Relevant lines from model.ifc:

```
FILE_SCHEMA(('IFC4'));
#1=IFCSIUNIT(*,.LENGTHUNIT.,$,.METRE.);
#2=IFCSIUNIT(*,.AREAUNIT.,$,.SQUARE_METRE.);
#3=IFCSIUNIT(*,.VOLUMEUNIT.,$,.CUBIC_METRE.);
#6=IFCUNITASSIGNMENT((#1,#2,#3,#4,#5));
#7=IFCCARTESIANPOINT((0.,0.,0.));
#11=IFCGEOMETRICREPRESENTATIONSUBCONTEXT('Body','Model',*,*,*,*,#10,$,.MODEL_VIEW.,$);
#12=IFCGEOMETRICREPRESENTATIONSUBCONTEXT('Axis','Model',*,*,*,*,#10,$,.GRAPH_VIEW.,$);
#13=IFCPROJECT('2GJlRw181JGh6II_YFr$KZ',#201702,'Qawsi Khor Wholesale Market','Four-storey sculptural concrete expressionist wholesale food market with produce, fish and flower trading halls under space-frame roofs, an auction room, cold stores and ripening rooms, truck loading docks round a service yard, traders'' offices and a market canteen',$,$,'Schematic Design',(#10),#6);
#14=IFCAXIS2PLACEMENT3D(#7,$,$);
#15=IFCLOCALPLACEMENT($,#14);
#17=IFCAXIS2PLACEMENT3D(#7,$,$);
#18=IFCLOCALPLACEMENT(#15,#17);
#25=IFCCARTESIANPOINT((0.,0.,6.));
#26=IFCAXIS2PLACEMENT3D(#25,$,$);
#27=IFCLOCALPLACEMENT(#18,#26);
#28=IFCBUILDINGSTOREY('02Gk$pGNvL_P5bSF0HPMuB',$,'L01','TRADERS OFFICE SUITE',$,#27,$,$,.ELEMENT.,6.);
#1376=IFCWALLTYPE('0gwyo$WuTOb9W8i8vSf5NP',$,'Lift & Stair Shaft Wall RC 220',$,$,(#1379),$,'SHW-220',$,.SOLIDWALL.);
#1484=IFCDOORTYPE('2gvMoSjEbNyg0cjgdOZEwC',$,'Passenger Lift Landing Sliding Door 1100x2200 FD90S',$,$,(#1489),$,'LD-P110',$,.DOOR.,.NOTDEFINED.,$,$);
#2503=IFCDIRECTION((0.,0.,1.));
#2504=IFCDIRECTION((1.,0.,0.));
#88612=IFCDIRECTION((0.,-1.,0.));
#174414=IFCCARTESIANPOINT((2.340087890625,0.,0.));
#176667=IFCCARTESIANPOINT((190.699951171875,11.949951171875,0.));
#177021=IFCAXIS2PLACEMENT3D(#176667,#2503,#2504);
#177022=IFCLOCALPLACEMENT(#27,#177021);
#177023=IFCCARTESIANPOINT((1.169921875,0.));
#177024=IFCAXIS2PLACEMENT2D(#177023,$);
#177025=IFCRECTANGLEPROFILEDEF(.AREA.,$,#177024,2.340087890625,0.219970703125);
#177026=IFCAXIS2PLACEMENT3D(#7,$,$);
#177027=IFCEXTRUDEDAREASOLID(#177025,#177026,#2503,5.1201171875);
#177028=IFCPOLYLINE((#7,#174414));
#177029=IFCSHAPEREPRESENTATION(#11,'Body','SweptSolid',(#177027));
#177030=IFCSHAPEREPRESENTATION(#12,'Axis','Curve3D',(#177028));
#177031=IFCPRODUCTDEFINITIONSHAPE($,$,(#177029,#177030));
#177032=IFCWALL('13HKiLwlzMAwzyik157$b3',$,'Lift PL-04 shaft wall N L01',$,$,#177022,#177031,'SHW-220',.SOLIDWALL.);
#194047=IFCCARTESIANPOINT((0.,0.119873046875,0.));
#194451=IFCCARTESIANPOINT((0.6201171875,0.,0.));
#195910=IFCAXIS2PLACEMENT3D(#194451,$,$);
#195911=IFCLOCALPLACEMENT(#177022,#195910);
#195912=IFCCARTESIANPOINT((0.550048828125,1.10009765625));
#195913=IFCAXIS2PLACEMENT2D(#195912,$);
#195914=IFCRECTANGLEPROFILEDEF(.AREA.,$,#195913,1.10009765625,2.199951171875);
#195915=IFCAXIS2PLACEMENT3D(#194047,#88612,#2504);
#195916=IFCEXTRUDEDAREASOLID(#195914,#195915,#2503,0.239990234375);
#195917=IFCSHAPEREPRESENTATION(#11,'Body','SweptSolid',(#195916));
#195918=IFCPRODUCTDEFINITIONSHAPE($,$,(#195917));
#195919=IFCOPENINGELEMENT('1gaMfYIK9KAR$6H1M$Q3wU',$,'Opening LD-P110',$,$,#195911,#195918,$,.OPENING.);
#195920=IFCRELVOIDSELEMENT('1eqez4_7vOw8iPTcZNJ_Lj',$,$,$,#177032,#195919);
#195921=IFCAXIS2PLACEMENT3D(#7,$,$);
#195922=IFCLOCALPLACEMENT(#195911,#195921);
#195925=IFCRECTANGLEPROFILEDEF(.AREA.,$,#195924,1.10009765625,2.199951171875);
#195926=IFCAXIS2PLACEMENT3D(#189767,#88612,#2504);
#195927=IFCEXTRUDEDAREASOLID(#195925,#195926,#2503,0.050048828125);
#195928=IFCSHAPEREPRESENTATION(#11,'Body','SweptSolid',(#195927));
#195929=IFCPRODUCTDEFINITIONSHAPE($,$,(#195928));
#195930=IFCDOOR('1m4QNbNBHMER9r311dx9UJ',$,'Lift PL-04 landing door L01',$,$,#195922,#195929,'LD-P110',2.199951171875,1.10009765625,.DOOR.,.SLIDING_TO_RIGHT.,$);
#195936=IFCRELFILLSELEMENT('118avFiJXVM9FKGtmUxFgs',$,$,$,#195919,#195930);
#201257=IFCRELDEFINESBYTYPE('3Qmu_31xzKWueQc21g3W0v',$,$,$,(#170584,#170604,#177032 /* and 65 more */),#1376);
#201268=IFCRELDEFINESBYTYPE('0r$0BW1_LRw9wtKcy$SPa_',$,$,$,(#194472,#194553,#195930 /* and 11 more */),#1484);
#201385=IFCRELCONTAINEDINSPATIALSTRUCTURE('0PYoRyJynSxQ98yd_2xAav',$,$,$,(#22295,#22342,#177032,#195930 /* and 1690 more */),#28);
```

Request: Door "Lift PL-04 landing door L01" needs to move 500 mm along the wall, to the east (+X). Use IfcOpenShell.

```python
import ifcopenshell
import ifcopenshell.api.geometry
import ifcopenshell.util.placement

model = ifcopenshell.open("model.ifc")

door = model.by_guid("1m4QNbNBHMER9r311dx9UJ")
opening = door.FillsVoids[0].RelatingOpeningElement
wall = opening.VoidsElements[0].RelatingBuildingElement

wall_matrix = ifcopenshell.util.placement.get_local_placement(wall.ObjectPlacement)
shift = wall_matrix[:3, 0] * 0.5
before = ifcopenshell.util.placement.get_local_placement(door.ObjectPlacement)[:3, 3].copy()

# The door is placed relative to its opening, so it follows when the opening moves.
matrix = ifcopenshell.util.placement.get_local_placement(opening.ObjectPlacement)
matrix[:3, 3] += shift
ifcopenshell.api.geometry.edit_object_placement(
    model, product=opening, matrix=matrix, is_si=False, should_transform_children=True
)

after = ifcopenshell.util.placement.get_local_placement(door.ObjectPlacement)[:3, 3]
print("door moved by", (after - before).round(3) + 0.0)

model.write("model_edited.ifc")
```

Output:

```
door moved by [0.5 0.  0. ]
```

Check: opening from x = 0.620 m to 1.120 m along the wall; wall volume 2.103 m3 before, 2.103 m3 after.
